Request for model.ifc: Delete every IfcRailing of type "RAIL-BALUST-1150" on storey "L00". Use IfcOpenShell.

First a look at what the model holds.

```python
import ifcopenshell
import ifcopenshell.util.element

model = ifcopenshell.open("model.ifc")
print(model.schema)
storey = next(s for s in model.by_type("IfcBuildingStorey") if s.Name == "L00")
railings = [e for e in ifcopenshell.util.element.get_decomposition(storey) if e.is_a("IfcRailing")]
seen = {}
for e in railings:
    element_type = ifcopenshell.util.element.get_type(e)
    name = element_type.Name if element_type not in (None, e) else None
    seen[name] = seen.get(name, 0) + 1
for name, count in sorted(seen.items(), key=str):
    print(count, "x", name)
```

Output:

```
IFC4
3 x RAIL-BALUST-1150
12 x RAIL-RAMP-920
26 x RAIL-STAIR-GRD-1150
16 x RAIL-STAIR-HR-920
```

```python
import ifcopenshell
import ifcopenshell.api.root
import ifcopenshell.util.element

model = ifcopenshell.open("model.ifc")

storey = next(s for s in model.by_type("IfcBuildingStorey") if s.Name == "L00")
railings = [e for e in ifcopenshell.util.element.get_decomposition(storey) if e.is_a("IfcRailing")]
targets = [e for e in railings if (t := ifcopenshell.util.element.get_type(e)) not in (None, e) and t.Name == "RAIL-BALUST-1150"]

for e in targets:
    ifcopenshell.api.root.remove_product(model, product=e)
print(len(targets), "removed")

model.write("model_rev.ifc")
```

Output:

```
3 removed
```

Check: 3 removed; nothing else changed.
